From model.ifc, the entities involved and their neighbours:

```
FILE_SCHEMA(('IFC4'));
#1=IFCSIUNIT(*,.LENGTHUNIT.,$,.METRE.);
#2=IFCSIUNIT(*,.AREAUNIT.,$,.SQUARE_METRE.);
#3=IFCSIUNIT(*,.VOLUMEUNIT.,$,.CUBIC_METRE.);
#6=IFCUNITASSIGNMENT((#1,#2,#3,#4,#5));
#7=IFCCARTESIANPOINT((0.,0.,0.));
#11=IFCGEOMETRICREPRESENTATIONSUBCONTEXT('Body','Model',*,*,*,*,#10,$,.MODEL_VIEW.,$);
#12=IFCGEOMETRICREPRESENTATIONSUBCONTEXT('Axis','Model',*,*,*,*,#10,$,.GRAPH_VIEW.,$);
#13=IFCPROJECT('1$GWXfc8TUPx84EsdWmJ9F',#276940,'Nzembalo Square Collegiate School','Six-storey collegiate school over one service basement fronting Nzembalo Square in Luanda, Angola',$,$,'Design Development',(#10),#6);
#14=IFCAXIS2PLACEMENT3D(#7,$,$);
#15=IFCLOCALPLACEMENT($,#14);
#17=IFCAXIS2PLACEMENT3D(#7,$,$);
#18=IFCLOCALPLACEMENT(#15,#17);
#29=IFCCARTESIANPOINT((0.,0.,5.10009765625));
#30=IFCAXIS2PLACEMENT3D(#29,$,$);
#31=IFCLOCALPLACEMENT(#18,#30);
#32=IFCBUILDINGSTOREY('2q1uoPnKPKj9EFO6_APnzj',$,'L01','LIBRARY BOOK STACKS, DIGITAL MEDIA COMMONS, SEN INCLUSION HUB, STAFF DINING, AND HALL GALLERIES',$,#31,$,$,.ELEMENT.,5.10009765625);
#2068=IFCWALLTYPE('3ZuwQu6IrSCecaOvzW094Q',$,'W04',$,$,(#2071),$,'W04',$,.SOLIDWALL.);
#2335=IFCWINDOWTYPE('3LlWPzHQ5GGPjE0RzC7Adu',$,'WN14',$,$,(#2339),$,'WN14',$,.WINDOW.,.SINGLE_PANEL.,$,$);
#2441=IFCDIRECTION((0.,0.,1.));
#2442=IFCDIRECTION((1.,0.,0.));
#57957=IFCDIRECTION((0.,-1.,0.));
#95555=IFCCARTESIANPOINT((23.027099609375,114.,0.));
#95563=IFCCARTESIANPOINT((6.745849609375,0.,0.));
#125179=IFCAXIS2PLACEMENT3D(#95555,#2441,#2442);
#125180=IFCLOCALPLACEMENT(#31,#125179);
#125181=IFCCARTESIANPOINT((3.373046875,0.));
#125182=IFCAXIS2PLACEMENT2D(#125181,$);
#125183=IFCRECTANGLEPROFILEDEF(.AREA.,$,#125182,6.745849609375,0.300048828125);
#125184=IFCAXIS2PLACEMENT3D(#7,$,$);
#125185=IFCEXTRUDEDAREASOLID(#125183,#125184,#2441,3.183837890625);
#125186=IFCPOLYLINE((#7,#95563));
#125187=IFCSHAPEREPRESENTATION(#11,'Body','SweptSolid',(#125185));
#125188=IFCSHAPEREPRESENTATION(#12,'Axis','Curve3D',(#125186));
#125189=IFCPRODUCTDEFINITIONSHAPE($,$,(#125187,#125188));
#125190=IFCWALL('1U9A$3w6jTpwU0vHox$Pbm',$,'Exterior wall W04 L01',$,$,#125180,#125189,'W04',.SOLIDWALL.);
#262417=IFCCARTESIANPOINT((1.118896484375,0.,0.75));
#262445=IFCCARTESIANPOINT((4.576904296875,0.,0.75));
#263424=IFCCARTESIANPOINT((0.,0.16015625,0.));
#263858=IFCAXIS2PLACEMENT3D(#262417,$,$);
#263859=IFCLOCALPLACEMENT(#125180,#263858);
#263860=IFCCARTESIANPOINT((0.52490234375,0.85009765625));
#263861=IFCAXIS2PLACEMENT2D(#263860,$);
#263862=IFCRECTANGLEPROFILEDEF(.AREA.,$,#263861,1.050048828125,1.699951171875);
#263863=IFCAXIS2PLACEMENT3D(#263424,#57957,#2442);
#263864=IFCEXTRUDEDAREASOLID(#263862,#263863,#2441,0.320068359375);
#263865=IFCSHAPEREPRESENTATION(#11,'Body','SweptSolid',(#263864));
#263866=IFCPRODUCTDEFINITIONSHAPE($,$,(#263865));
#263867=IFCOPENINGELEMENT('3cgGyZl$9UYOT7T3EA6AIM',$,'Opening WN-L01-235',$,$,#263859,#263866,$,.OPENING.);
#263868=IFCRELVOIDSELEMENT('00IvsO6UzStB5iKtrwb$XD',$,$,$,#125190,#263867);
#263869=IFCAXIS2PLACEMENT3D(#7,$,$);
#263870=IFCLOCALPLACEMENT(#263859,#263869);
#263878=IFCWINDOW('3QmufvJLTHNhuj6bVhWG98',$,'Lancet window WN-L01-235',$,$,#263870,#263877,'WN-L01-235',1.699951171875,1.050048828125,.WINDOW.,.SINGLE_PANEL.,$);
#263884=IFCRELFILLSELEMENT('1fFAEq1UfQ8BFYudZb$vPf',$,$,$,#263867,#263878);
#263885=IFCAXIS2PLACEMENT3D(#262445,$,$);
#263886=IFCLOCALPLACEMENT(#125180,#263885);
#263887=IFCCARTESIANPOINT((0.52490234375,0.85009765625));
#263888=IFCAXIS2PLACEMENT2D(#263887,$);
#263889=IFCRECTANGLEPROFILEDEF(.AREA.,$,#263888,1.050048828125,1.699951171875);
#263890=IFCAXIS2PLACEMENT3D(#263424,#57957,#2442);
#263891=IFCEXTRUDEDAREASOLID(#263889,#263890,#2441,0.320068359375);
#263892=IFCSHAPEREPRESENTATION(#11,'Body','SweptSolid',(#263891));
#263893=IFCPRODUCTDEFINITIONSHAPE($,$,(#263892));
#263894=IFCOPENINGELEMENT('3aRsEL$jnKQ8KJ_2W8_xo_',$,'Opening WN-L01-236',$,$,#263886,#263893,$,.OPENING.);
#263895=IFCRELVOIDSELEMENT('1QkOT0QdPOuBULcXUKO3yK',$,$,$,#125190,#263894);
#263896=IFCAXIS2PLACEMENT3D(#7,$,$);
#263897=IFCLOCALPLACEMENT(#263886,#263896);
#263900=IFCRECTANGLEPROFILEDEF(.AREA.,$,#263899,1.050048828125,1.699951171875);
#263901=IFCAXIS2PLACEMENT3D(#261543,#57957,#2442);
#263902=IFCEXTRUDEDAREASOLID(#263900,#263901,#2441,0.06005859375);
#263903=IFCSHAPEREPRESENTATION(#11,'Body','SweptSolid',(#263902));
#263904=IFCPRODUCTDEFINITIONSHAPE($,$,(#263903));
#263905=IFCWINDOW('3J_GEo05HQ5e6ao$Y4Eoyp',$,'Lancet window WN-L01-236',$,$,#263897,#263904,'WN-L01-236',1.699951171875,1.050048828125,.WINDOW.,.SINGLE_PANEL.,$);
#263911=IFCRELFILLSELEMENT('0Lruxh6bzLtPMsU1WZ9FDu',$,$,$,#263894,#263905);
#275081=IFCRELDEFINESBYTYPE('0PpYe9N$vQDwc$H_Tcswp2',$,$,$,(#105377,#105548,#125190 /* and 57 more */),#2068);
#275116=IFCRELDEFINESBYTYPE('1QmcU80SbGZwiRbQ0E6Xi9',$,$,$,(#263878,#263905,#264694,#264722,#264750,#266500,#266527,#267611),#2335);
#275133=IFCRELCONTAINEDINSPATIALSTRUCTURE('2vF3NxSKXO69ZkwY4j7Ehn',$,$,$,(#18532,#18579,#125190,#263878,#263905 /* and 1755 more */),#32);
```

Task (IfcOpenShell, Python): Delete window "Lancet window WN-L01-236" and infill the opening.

```python
import ifcopenshell
import ifcopenshell.api.feature
import ifcopenshell.api.root
import ifcopenshell.geom
import ifcopenshell.util.shape

model = ifcopenshell.open("model.ifc")
settings = ifcopenshell.geom.settings()


def volume(element):
    """Net volume in cubic metres, openings subtracted."""
    shape = ifcopenshell.geom.create_shape(settings, element)
    return ifcopenshell.util.shape.get_volume(shape.geometry)


window = model.by_guid("3J_GEo05HQ5e6ao$Y4Eoyp")
opening = window.FillsVoids[0].RelatingOpeningElement
wall = opening.VoidsElements[0].RelatingBuildingElement
before = volume(wall)

ifcopenshell.api.root.remove_product(model, product=window)
ifcopenshell.api.feature.remove_feature(model, feature=opening)

after = volume(wall)

print(f"wall volume {before:.3f} -> {after:.3f} m3")

model.write("model_v2.ifc")
```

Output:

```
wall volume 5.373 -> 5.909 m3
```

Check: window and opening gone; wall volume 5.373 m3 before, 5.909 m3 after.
